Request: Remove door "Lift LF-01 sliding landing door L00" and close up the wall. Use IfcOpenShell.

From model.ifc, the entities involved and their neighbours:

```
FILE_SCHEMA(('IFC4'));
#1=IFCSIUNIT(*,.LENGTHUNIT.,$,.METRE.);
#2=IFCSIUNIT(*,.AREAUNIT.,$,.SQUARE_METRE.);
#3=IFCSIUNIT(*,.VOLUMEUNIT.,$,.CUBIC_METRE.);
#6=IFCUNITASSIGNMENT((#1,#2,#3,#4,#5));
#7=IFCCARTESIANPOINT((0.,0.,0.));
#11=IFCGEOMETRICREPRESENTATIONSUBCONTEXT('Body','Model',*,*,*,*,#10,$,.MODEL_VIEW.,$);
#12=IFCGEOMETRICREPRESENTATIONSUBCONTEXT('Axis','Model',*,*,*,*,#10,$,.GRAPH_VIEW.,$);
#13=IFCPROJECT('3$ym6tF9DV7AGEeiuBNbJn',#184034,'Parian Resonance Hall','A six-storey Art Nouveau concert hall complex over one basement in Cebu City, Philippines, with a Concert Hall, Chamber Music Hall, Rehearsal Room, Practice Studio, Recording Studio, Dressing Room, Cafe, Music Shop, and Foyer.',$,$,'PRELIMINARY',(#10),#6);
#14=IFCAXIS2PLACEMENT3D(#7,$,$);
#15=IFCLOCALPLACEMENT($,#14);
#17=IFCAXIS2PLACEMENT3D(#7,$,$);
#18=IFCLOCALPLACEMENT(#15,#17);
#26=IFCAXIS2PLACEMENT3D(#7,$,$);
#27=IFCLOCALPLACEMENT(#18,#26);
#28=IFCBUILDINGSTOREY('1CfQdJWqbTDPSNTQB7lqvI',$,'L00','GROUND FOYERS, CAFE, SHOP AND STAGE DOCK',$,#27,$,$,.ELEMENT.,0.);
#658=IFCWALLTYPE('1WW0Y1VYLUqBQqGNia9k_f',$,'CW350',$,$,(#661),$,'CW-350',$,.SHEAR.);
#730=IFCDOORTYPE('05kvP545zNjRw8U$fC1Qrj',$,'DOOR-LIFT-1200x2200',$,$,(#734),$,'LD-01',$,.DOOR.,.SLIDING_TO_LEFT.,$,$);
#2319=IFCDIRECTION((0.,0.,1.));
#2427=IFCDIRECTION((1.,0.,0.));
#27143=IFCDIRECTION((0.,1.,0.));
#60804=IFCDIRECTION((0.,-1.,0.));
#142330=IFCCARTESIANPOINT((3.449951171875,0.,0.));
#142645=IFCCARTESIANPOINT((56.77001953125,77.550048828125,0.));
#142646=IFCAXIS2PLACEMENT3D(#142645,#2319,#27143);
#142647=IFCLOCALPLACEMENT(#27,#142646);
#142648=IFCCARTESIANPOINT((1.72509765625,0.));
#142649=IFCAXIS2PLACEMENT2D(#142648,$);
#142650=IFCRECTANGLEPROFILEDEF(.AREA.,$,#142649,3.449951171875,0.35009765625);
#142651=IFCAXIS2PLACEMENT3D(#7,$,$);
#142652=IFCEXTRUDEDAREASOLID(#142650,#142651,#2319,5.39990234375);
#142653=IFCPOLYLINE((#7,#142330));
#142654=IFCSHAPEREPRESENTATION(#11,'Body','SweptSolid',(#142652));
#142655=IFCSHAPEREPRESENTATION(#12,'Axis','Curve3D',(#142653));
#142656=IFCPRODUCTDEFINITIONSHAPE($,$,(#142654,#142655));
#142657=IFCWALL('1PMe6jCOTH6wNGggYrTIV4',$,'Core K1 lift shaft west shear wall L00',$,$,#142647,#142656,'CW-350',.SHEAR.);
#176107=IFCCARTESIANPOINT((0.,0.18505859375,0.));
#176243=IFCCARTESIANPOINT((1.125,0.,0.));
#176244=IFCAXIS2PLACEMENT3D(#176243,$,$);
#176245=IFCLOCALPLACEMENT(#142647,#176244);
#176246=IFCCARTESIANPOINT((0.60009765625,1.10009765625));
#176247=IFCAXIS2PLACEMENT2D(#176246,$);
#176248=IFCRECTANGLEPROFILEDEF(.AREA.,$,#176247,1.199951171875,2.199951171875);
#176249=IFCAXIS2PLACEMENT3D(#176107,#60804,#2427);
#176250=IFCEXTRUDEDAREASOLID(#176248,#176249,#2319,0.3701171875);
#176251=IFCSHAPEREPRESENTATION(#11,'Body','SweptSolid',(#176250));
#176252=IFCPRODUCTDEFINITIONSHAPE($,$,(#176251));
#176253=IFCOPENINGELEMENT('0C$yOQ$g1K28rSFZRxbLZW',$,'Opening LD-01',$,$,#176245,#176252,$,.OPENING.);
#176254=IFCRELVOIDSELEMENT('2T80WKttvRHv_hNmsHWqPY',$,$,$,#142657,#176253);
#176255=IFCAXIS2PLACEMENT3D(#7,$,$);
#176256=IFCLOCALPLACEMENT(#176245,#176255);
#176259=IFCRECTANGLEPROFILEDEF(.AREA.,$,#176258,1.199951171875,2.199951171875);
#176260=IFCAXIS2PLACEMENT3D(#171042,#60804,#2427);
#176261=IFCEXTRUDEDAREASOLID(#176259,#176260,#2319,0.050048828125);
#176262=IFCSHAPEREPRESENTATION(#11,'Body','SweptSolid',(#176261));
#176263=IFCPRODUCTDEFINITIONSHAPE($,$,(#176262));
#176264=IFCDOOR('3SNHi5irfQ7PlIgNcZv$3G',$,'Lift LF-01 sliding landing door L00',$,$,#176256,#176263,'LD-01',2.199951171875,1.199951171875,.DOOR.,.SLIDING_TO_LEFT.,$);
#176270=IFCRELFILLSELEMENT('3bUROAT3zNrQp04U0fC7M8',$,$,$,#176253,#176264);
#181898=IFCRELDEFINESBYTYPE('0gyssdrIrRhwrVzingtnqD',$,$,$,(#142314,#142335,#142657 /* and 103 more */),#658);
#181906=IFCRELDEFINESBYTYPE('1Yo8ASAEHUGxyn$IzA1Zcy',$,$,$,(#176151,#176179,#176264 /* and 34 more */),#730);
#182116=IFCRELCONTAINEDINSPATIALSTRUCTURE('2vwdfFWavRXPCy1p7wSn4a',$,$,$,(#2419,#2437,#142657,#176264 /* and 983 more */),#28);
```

```python
import ifcopenshell
import ifcopenshell.api.feature
import ifcopenshell.api.root
import ifcopenshell.geom
import ifcopenshell.util.shape

model = ifcopenshell.open("model.ifc")
settings = ifcopenshell.geom.settings()


def volume(element):
    """Net volume in cubic metres, openings subtracted."""
    shape = ifcopenshell.geom.create_shape(settings, element)
    return ifcopenshell.util.shape.get_volume(shape.geometry)


door = model.by_guid("3SNHi5irfQ7PlIgNcZv$3G")
opening = door.FillsVoids[0].RelatingOpeningElement
wall = opening.VoidsElements[0].RelatingBuildingElement
before = volume(wall)

ifcopenshell.api.root.remove_product(model, product=door)
ifcopenshell.api.feature.remove_feature(model, feature=opening)

after = volume(wall)

print(f"wall volume {before:.3f} -> {after:.3f} m3")

model.write("model-out.ifc")
```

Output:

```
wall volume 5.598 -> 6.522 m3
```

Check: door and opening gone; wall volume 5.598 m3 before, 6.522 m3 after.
